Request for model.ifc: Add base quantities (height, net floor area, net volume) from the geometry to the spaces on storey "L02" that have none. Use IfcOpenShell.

First a look at what the model holds.

```python
import ifcopenshell
import ifcopenshell.util.element
import ifcopenshell.util.unit

model = ifcopenshell.open("model.ifc")
print(model.schema)
for unit_type in ("LENGTHUNIT", "AREAUNIT", "VOLUMEUNIT"):
    print(unit_type, ifcopenshell.util.unit.calculate_unit_scale(model, unit_type))
storey = next(s for s in model.by_type("IfcBuildingStorey") if s.Name == "L02")
spaces = [e for e in ifcopenshell.util.element.get_decomposition(storey) if e.is_a("IfcSpace")]
for e in sorted(spaces, key=lambda e: e.id()):
    print(e.id(), e.is_a(), e.Name, list(ifcopenshell.util.element.get_psets(e, qtos_only=True)), sep=" | ")
```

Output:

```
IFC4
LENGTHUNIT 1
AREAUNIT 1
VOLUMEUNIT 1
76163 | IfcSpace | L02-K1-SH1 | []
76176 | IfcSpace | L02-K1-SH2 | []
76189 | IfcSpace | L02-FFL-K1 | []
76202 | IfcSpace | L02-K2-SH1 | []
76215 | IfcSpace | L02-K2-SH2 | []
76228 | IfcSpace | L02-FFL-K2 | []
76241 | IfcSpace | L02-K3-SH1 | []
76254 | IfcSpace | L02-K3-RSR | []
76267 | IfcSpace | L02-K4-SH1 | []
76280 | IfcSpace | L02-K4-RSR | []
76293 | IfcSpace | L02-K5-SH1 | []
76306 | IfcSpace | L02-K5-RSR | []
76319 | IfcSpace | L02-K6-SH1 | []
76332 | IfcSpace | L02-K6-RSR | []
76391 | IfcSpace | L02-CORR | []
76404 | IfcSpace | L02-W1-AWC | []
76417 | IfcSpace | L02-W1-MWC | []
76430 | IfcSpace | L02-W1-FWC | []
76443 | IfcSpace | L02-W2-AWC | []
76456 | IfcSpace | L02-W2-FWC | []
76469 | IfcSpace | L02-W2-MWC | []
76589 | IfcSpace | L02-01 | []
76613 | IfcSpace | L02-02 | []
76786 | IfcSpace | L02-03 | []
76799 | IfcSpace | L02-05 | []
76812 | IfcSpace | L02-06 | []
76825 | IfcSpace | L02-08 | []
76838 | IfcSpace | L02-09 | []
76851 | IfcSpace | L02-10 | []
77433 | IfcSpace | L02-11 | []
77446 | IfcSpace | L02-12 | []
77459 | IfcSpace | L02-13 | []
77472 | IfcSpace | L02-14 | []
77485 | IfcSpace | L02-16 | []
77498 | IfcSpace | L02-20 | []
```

```python
import ifcopenshell
import ifcopenshell.api.pset
import ifcopenshell.geom
import ifcopenshell.util.element
import ifcopenshell.util.shape
import ifcopenshell.util.unit

model = ifcopenshell.open("model.ifc")
unit_scale = ifcopenshell.util.unit.calculate_unit_scale(model)
area_scale = ifcopenshell.util.unit.calculate_unit_scale(model, "AREAUNIT")
volume_scale = ifcopenshell.util.unit.calculate_unit_scale(model, "VOLUMEUNIT")
settings = ifcopenshell.geom.settings()

storey = next(s for s in model.by_type("IfcBuildingStorey") if s.Name == "L02")
spaces = [e for e in ifcopenshell.util.element.get_decomposition(storey) if e.is_a("IfcSpace")]

for e in sorted(spaces, key=lambda e: e.id()):
    if ifcopenshell.util.element.get_psets(e, qtos_only=True, should_inherit=False):
        continue
    # Geometry comes back in metres, in the element's own axes.
    shape = ifcopenshell.geom.create_shape(settings, e)
    values = {
        "Height": ifcopenshell.util.shape.get_z(shape.geometry) / unit_scale,
        "NetFloorArea": ifcopenshell.util.shape.get_footprint_area(shape.geometry) / area_scale,
        "NetVolume": ifcopenshell.util.shape.get_volume(shape.geometry) / volume_scale,
    }
    qto = ifcopenshell.api.pset.add_qto(model, product=e, name="Qto_SpaceBaseQuantities")
    ifcopenshell.api.pset.edit_qto(model, qto=qto, properties=values)
    print(e.id(), {k: round(v, 3) for k, v in values.items()})

model.write("model_updated.ifc")
```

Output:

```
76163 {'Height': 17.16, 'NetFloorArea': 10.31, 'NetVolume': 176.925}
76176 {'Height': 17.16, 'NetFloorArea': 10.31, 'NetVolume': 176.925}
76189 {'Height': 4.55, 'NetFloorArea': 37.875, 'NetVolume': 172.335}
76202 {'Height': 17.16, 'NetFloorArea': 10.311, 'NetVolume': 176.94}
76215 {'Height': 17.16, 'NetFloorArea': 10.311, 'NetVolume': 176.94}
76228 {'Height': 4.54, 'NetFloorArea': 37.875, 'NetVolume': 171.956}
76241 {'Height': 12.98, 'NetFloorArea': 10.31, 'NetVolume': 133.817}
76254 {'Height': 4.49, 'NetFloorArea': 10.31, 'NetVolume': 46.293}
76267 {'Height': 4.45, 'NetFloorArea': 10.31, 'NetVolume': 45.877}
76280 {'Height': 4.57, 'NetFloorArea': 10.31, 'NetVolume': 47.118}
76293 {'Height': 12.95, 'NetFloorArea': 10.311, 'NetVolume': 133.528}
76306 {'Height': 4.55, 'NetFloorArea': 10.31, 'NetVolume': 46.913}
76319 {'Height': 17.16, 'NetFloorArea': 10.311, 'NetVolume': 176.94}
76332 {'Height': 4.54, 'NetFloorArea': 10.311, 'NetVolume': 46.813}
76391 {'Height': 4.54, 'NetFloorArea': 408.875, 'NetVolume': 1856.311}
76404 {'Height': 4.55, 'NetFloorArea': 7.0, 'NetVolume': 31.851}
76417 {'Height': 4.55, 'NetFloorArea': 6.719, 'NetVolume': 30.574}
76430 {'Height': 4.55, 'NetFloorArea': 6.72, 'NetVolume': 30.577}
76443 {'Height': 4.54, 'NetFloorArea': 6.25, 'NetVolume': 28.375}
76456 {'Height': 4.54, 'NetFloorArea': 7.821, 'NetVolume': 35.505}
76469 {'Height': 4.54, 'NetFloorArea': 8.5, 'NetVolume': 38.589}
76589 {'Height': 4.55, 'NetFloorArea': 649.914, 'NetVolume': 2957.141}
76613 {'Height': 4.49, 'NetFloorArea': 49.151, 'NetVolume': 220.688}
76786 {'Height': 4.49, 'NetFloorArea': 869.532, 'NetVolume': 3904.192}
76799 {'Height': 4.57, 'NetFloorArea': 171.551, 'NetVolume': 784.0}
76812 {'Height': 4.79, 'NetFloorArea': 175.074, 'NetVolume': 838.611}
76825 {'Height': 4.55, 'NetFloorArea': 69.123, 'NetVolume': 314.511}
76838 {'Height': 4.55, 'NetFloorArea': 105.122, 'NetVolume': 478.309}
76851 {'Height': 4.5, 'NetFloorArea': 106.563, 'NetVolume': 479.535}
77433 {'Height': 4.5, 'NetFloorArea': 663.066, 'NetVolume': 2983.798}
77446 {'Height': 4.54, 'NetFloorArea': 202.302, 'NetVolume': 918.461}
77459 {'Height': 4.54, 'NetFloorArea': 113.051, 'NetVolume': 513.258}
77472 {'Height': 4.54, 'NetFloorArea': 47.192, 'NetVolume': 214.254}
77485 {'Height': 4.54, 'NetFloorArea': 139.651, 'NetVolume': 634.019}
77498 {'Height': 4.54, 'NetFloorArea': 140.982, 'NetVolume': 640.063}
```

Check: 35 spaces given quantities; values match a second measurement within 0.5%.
